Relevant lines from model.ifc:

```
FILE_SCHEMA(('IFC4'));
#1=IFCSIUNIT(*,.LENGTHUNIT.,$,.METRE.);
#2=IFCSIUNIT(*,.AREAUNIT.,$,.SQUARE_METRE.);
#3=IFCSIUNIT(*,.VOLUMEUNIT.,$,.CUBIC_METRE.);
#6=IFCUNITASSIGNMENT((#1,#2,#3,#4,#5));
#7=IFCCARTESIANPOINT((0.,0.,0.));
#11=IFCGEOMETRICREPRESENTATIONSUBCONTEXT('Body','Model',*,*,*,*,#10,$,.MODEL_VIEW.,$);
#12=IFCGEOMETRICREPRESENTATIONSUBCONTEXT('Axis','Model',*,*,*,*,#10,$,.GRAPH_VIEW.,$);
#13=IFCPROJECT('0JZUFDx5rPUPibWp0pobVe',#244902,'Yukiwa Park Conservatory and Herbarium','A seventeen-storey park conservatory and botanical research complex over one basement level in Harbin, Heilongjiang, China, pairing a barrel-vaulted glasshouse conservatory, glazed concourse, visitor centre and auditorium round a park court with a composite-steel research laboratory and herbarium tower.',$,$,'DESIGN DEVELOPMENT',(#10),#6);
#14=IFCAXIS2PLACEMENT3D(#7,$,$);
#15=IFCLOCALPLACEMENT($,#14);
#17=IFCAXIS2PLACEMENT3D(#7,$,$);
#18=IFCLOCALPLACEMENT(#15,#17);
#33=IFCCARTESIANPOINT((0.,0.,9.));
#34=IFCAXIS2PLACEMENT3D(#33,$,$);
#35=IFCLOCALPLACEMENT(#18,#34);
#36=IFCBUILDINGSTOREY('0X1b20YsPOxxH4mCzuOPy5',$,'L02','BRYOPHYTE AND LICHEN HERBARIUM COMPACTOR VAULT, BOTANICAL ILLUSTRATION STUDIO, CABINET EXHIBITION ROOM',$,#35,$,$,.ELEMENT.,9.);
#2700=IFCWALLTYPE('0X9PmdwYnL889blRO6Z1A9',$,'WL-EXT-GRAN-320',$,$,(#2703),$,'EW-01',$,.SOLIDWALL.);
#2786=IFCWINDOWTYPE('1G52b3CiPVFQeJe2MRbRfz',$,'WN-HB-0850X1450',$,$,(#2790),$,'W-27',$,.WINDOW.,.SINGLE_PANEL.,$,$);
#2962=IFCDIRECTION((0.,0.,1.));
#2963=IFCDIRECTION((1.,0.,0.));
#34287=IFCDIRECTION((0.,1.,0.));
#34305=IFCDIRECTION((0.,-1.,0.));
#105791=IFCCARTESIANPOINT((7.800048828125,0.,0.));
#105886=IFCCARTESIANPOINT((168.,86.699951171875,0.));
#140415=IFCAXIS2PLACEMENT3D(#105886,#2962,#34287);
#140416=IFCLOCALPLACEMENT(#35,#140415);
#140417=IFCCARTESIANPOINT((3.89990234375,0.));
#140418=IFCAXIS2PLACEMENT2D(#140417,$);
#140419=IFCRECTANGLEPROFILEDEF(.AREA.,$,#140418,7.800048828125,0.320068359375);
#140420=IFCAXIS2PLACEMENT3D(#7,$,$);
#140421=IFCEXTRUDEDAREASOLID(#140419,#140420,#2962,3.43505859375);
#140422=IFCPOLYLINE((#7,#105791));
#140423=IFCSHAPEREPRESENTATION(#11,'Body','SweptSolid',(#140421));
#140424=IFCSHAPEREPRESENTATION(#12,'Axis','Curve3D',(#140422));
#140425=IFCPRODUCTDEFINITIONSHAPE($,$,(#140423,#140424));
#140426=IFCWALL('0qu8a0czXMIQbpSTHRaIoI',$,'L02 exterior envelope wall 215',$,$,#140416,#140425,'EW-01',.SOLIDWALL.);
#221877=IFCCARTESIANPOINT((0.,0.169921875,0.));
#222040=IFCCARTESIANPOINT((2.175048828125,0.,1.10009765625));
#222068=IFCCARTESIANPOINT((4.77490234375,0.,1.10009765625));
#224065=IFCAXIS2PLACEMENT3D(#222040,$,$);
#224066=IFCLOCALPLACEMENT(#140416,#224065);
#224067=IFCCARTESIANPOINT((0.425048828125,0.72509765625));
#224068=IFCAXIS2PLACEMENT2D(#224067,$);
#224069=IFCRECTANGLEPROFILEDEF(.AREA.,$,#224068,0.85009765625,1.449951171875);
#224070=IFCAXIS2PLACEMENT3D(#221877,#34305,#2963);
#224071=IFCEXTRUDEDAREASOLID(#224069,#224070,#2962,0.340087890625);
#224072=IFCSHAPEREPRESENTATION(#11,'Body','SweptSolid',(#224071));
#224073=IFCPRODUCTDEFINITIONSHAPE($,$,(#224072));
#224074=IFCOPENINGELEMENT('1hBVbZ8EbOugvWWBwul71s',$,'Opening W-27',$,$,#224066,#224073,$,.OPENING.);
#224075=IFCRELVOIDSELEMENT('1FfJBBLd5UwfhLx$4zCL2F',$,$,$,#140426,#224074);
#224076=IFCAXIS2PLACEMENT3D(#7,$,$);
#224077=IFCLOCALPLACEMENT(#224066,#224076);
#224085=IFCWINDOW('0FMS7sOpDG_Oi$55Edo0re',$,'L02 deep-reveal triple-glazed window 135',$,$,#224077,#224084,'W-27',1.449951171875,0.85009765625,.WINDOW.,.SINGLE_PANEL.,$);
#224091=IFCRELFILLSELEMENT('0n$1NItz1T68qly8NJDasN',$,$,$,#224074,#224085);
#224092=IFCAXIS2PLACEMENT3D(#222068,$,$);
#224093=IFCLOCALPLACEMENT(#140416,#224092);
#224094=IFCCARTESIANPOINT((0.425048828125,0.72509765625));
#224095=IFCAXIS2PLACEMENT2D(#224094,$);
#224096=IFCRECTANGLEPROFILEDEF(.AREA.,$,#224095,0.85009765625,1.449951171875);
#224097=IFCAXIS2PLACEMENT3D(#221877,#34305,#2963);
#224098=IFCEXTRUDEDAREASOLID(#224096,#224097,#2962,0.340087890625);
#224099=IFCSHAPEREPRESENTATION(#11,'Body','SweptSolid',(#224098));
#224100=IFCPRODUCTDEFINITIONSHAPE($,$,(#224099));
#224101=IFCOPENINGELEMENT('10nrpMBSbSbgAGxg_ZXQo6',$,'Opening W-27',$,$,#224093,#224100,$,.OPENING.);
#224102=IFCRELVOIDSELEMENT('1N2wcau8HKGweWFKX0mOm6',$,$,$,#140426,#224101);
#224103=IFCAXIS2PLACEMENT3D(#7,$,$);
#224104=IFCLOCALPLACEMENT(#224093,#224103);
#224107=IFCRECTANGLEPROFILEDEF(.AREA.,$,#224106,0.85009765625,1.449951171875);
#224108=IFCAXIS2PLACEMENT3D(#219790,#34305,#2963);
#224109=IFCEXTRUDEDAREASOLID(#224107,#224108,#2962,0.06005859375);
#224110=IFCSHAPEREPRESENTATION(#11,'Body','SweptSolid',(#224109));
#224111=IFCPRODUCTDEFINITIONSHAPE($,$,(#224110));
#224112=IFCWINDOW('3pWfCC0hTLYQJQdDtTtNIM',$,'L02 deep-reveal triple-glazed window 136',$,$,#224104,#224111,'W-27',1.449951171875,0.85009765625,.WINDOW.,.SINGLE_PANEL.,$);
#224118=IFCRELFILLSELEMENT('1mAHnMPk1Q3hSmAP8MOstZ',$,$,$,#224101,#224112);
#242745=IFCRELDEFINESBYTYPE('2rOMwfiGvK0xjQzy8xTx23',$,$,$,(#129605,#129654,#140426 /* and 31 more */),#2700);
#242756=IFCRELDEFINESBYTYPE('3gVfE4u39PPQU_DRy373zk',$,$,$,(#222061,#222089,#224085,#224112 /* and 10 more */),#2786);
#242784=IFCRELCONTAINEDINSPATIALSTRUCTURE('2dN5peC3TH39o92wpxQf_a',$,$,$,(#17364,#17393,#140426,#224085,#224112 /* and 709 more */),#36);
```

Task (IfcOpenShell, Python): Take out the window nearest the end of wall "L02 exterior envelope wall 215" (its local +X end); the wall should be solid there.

```python
import ifcopenshell
import ifcopenshell.api.feature
import ifcopenshell.api.root
import ifcopenshell.geom
import ifcopenshell.util.shape

model = ifcopenshell.open("model.ifc")
settings = ifcopenshell.geom.settings()


def volume(element):
    """Net volume in cubic metres, openings subtracted."""
    shape = ifcopenshell.geom.create_shape(settings, element)
    return ifcopenshell.util.shape.get_volume(shape.geometry)


window = model.by_id(224112)
opening = window.FillsVoids[0].RelatingOpeningElement
wall = opening.VoidsElements[0].RelatingBuildingElement
before = volume(wall)

ifcopenshell.api.root.remove_product(model, product=window)
ifcopenshell.api.feature.remove_feature(model, feature=opening)

after = volume(wall)

print(f"wall volume {before:.3f} -> {after:.3f} m3")

model.write("model_updated.ifc")
```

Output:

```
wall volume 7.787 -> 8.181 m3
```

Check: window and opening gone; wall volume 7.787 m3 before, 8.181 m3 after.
